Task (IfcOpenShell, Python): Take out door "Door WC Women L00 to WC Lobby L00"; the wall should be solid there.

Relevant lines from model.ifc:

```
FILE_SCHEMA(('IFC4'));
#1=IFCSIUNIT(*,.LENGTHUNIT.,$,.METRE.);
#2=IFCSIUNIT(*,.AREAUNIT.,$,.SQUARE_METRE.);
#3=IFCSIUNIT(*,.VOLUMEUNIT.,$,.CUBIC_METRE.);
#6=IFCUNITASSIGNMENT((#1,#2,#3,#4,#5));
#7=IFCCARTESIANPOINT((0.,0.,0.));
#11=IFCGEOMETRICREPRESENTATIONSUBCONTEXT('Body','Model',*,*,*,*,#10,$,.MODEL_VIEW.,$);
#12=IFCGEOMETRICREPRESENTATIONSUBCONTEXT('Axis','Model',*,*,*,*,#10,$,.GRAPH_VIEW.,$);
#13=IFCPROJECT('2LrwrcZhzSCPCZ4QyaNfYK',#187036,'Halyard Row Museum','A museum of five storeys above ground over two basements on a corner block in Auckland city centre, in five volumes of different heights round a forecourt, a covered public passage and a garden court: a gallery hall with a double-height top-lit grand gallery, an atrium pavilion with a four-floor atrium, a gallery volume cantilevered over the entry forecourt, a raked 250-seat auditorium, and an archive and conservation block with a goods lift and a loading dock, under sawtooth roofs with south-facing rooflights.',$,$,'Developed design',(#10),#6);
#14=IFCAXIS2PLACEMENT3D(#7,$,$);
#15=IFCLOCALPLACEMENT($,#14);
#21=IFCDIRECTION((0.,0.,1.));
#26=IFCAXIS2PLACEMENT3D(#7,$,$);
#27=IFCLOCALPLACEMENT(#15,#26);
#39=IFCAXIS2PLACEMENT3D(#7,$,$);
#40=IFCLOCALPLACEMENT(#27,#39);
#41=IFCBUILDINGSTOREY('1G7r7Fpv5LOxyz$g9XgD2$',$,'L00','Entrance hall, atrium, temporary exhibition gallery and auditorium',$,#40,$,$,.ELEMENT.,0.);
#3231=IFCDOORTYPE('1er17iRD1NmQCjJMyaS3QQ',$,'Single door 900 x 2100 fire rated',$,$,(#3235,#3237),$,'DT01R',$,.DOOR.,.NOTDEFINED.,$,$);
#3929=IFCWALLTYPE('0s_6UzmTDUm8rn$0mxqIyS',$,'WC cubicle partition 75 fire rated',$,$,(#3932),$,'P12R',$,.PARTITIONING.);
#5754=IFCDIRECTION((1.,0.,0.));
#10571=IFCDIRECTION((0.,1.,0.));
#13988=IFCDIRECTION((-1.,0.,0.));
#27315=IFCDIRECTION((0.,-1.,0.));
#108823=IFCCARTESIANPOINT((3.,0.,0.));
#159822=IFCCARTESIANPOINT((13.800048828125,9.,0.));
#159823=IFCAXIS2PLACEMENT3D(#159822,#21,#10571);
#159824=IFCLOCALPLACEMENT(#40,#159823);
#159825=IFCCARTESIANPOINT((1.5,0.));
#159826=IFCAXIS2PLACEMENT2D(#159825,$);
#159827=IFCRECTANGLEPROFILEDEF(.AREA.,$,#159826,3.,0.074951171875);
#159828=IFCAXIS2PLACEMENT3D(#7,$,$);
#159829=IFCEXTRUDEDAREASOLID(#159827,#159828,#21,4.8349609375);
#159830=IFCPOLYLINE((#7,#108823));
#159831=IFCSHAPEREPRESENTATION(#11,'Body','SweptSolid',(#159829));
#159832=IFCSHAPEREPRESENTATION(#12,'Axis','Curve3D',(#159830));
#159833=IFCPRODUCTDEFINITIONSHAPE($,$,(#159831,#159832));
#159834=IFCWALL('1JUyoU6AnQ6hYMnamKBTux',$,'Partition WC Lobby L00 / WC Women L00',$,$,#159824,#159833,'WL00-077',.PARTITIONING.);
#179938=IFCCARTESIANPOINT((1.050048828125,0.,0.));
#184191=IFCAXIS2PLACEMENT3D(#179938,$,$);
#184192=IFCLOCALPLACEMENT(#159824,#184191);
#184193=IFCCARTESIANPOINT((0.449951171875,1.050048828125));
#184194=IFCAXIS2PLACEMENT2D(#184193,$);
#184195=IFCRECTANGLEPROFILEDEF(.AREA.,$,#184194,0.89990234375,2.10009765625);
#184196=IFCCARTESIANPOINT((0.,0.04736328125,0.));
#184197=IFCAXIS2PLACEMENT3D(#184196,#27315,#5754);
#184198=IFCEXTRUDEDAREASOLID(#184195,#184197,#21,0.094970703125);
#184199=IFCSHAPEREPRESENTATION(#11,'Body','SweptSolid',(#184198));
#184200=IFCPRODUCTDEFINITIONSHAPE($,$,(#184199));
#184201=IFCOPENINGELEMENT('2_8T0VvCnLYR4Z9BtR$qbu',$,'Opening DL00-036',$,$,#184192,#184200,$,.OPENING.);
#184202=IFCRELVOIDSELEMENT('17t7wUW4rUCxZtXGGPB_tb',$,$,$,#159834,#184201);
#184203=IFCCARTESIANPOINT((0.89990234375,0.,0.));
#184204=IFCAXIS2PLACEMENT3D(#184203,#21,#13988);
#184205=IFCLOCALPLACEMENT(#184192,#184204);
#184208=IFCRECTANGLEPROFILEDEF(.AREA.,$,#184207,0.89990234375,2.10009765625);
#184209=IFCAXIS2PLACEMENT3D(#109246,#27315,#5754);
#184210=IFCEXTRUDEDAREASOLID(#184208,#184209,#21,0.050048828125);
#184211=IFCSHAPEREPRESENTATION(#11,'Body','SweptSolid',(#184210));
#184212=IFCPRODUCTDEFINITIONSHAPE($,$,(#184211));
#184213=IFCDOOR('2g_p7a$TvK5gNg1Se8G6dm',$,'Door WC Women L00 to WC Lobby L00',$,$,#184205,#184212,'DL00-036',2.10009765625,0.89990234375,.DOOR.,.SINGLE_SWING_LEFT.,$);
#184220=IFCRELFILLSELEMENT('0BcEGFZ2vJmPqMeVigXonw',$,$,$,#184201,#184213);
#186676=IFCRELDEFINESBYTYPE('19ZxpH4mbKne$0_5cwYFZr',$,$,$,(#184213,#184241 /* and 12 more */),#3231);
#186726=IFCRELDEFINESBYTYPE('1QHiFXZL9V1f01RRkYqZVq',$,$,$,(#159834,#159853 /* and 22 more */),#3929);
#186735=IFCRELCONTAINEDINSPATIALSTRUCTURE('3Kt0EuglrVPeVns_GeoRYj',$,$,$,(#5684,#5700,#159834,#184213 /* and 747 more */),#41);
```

```python
import ifcopenshell
import ifcopenshell.api.feature
import ifcopenshell.api.root
import ifcopenshell.geom
import ifcopenshell.util.shape

model = ifcopenshell.open("model.ifc")
settings = ifcopenshell.geom.settings()


def volume(element):
    """Net volume in cubic metres, openings subtracted."""
    shape = ifcopenshell.geom.create_shape(settings, element)
    return ifcopenshell.util.shape.get_volume(shape.geometry)


door = model.by_id(184213)
opening = door.FillsVoids[0].RelatingOpeningElement
wall = opening.VoidsElements[0].RelatingBuildingElement
before = volume(wall)

ifcopenshell.api.root.remove_product(model, product=door)
ifcopenshell.api.feature.remove_feature(model, feature=opening)

after = volume(wall)

print(f"wall volume {before:.3f} -> {after:.3f} m3")

model.write("model_edited.ifc")
```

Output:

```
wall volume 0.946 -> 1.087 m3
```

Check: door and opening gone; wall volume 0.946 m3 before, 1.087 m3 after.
